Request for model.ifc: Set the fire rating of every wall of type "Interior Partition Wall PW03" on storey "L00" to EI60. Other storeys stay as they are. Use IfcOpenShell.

First a look at what the model holds.

```python
import ifcopenshell
import ifcopenshell.util.element

model = ifcopenshell.open("model.ifc")
print(model.schema)
storey = next(s for s in model.by_type("IfcBuildingStorey") if s.Name == "L00")
walls = [e for e in ifcopenshell.util.element.get_decomposition(storey) if e.is_a("IfcWall")]
seen = {}
for e in walls:
    element_type = ifcopenshell.util.element.get_type(e)
    key = (element_type.Name if element_type != e and element_type else None, ifcopenshell.util.element.get_pset(e, "Pset_WallCommon", "FireRating"))
    seen[key] = seen.get(key, 0) + 1
for (name, value), count in sorted(seen.items(), key=str):
    print(count, "x", name, "|", value)
```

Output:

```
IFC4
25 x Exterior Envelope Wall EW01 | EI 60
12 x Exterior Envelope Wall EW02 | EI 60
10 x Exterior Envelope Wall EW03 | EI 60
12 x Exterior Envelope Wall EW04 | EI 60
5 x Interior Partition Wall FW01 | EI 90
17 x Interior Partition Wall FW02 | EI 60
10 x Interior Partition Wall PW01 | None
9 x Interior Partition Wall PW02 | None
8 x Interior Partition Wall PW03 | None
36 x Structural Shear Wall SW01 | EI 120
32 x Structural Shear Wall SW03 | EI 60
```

```python
import ifcopenshell
import ifcopenshell.api.pset
import ifcopenshell.util.element

model = ifcopenshell.open("model.ifc")

storey = next(s for s in model.by_type("IfcBuildingStorey") if s.Name == "L00")
walls = [e for e in ifcopenshell.util.element.get_decomposition(storey) if e.is_a("IfcWall")]

count = 0
for e in walls:
    element_type = ifcopenshell.util.element.get_type(e)
    if element_type in (None, e) or element_type.Name != "Interior Partition Wall PW03":
        continue
    # add_pset returns the element's existing set when there is one.
    pset = ifcopenshell.api.pset.add_pset(model, product=e, name="Pset_WallCommon")
    ifcopenshell.api.pset.edit_pset(model, pset=pset, properties={"FireRating": "EI60"})
    count += 1

print(count, "walls updated")

model.write("model_edited.ifc")
```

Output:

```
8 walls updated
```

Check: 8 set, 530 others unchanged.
